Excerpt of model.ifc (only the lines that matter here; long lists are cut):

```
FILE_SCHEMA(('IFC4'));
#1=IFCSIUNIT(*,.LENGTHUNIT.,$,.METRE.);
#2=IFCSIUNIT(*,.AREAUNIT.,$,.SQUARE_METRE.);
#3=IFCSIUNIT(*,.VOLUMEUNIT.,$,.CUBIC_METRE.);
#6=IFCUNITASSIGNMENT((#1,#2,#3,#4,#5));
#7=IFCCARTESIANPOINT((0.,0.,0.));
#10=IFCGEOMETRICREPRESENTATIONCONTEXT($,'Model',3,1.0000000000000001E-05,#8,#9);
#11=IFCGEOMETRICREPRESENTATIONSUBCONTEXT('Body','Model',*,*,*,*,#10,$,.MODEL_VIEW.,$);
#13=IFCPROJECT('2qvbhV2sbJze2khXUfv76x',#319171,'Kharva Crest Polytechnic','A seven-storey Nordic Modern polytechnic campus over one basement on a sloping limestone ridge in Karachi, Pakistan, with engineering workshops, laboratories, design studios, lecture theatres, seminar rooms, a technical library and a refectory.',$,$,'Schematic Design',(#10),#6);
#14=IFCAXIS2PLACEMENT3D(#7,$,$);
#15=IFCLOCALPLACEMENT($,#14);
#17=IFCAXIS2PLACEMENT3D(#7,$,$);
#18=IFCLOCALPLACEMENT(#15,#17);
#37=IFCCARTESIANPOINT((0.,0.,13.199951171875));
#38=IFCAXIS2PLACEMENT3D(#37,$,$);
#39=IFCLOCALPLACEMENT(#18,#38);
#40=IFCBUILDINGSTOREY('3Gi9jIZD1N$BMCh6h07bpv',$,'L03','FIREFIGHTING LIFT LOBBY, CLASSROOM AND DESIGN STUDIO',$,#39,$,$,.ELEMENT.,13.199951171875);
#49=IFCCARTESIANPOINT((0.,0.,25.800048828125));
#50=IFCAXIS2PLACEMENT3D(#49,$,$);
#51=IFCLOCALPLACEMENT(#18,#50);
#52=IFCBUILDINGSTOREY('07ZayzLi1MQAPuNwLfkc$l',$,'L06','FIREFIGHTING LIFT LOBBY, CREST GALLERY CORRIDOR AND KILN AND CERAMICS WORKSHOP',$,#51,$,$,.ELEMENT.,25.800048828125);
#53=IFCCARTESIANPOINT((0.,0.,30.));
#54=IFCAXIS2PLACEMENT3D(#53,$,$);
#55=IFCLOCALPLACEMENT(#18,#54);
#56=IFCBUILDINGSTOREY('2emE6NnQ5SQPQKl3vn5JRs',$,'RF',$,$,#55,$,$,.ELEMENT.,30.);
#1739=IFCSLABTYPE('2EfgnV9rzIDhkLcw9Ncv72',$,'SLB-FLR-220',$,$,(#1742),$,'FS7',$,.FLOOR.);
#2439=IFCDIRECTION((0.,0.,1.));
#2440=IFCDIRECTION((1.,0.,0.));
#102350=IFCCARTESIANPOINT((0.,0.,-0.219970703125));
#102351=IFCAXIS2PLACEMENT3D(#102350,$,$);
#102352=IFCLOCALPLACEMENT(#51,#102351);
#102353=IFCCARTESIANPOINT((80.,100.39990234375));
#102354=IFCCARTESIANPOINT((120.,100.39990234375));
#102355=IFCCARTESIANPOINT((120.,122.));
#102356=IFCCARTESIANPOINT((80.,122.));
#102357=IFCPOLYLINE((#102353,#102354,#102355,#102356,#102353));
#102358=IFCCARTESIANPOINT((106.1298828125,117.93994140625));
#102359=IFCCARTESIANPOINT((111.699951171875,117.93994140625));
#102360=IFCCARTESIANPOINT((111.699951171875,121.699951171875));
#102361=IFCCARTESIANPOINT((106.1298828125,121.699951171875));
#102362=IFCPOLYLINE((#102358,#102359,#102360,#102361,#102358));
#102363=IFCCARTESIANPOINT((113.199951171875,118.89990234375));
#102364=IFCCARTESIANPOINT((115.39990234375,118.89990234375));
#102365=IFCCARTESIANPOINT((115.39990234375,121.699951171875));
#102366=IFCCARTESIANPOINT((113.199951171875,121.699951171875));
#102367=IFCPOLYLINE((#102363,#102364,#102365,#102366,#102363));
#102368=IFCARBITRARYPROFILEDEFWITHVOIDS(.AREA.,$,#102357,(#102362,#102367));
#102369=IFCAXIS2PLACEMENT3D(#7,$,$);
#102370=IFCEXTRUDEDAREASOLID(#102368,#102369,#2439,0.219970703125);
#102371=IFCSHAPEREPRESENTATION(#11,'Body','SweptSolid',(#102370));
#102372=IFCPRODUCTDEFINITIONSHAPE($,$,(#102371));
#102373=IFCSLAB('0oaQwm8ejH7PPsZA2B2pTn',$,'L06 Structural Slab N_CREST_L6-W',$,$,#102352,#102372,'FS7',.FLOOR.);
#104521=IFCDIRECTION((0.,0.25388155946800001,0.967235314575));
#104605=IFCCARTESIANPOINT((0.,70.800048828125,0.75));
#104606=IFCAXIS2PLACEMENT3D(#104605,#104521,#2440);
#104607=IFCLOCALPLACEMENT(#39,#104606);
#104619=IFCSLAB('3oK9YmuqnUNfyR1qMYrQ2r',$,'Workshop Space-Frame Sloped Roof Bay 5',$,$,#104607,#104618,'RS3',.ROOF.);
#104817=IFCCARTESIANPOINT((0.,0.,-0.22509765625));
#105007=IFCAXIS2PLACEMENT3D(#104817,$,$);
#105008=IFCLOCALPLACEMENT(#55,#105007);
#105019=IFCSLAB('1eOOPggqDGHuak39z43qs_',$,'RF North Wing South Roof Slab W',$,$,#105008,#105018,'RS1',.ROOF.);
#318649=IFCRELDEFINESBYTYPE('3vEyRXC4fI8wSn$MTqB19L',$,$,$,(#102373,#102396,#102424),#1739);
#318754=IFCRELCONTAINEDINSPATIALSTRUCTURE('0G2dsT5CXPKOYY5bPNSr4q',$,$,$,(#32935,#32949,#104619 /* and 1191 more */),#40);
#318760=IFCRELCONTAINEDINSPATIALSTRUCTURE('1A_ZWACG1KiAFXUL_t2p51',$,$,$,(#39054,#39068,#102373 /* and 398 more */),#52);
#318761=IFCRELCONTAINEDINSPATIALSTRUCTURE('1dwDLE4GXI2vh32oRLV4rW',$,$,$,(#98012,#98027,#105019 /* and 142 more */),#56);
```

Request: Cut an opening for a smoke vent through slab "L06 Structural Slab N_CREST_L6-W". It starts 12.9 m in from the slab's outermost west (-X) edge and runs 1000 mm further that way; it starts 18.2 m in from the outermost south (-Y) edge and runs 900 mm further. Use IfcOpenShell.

```python
import numpy as np
import ifcopenshell
import ifcopenshell.api.feature
import ifcopenshell.api.geometry
import ifcopenshell.api.root
import ifcopenshell.geom
import ifcopenshell.util.placement
import ifcopenshell.util.representation
import ifcopenshell.util.shape
import ifcopenshell.util.unit

model = ifcopenshell.open("model.ifc")
unit_scale = ifcopenshell.util.unit.calculate_unit_scale(model)
settings = ifcopenshell.geom.settings()


def volume(element):
    """Net volume in cubic metres, openings subtracted."""
    shape = ifcopenshell.geom.create_shape(settings, element)
    return ifcopenshell.util.shape.get_volume(shape.geometry)


slab = model.by_guid("0oaQwm8ejH7PPsZA2B2pTn")
before = volume(slab)

# Extent in the slab's own axes, in metres. The edges named are its -X and -Y sides.
slab_shape = ifcopenshell.geom.create_shape(settings, slab)
vertices = ifcopenshell.util.shape.get_vertices(slab_shape.geometry)
x_min, y_min, bottom = vertices.min(axis=0)
top = vertices[:, 2].max()

opening = ifcopenshell.api.root.create_entity(model, ifc_class="IfcOpeningElement", name="Smoke vent opening", predefined_type="OPENING")
context = ifcopenshell.util.representation.get_context(model, "Model", "Body", "MODEL_VIEW")
width, depth = 1, 0.9
outline = [(0.0, 0.0), (width, 0.0), (width, depth), (0.0, depth), (0.0, 0.0)]
# Overshoot both faces by 50 mm so the cut is clean.
shape = ifcopenshell.api.geometry.add_slab_representation(
    model, context=context, depth=top - bottom + 0.1, polyline=outline
)
ifcopenshell.api.geometry.assign_representation(model, product=opening, representation=shape)

matrix = ifcopenshell.util.placement.get_local_placement(slab.ObjectPlacement)
matrix[:, 3] = matrix @ np.append(np.array([x_min + 12.9, y_min + 18.2, bottom - 0.05]) / unit_scale, 1.0)
ifcopenshell.api.geometry.edit_object_placement(model, product=opening, matrix=matrix, is_si=False)
ifcopenshell.api.feature.add_feature(model, feature=opening, element=slab)

after = volume(slab)

print(f"slab volume {before:.3f} -> {after:.3f} m3")

model.write("model-out.ifc")
```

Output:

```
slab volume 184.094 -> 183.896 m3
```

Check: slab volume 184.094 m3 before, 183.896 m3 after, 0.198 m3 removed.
